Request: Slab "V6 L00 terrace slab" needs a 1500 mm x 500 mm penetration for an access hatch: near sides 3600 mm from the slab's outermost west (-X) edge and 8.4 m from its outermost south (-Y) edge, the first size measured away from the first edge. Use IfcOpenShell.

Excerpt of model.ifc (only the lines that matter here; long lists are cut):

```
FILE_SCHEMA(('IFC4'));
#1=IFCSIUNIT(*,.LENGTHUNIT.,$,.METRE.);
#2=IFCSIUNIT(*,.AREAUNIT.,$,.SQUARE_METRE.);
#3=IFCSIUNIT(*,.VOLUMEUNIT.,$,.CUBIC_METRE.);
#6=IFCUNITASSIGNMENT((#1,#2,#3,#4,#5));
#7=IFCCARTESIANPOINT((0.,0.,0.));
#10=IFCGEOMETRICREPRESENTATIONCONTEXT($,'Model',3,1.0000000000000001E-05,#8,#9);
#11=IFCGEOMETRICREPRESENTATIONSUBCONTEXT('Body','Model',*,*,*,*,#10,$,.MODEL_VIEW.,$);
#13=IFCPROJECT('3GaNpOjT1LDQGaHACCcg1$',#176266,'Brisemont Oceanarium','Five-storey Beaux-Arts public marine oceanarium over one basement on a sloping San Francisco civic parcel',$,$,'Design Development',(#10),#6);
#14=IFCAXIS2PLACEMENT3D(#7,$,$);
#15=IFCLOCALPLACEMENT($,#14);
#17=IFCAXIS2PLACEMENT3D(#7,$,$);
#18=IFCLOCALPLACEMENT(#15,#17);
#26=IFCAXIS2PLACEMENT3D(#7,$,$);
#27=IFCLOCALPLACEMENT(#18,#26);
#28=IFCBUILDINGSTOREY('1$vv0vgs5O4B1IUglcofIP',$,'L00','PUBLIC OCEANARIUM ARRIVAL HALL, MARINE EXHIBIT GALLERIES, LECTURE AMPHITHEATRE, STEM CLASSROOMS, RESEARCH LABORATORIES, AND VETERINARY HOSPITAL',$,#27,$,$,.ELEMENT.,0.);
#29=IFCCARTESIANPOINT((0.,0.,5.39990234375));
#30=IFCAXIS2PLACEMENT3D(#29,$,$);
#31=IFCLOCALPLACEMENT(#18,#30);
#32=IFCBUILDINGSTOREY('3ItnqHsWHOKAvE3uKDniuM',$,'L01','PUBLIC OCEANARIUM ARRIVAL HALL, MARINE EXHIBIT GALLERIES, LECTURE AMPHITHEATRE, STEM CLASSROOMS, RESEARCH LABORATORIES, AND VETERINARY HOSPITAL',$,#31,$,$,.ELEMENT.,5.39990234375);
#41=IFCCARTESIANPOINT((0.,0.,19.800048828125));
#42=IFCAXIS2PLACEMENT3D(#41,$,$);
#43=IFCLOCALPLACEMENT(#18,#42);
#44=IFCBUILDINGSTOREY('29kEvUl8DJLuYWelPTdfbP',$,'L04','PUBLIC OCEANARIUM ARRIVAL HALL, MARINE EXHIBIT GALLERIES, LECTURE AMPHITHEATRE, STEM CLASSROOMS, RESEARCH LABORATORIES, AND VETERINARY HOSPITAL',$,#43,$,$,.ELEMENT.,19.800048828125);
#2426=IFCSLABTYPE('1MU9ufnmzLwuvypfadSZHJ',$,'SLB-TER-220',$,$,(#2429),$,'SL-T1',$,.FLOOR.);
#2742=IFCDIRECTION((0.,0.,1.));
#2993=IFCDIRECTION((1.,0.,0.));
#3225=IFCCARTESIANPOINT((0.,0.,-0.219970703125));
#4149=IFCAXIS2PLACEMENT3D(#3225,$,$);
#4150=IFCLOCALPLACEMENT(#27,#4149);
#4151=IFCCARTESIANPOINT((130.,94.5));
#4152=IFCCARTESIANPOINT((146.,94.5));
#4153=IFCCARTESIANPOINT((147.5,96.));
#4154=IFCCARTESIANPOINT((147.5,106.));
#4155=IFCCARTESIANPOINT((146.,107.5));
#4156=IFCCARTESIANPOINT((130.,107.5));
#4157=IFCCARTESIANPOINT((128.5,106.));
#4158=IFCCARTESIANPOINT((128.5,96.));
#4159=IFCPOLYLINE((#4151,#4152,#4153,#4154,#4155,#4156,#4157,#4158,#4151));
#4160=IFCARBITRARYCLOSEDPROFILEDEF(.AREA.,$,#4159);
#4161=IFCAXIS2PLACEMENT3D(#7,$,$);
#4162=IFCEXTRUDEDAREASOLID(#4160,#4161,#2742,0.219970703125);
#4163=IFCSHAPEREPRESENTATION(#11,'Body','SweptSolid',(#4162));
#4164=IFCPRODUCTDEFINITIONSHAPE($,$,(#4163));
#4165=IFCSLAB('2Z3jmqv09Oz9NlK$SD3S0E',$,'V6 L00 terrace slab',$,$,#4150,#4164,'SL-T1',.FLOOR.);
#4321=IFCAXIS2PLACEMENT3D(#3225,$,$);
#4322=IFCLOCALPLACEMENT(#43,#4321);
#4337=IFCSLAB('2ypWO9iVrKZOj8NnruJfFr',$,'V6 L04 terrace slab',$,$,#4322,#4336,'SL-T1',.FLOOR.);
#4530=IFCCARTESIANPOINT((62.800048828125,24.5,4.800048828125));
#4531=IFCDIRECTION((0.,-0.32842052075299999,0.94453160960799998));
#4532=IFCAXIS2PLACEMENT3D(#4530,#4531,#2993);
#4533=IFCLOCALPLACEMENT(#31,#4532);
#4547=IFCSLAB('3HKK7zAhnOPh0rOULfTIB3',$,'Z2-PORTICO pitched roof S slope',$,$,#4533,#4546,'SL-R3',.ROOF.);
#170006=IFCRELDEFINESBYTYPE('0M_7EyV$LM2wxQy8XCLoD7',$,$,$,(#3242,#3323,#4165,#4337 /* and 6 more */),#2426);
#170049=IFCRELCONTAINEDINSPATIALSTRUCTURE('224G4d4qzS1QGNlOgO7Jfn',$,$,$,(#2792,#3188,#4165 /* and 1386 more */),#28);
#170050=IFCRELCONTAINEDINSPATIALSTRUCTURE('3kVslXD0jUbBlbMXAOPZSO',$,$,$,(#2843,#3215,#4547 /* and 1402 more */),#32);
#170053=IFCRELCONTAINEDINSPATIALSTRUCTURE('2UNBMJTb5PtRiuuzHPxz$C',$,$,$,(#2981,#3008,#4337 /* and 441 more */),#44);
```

```python
import numpy as np
import ifcopenshell
import ifcopenshell.api.feature
import ifcopenshell.api.geometry
import ifcopenshell.api.root
import ifcopenshell.geom
import ifcopenshell.util.placement
import ifcopenshell.util.representation
import ifcopenshell.util.shape
import ifcopenshell.util.unit

model = ifcopenshell.open("model.ifc")
unit_scale = ifcopenshell.util.unit.calculate_unit_scale(model)
settings = ifcopenshell.geom.settings()


def volume(element):
    """Net volume in cubic metres, openings subtracted."""
    shape = ifcopenshell.geom.create_shape(settings, element)
    return ifcopenshell.util.shape.get_volume(shape.geometry)


slab = model.by_guid("2Z3jmqv09Oz9NlK$SD3S0E")
before = volume(slab)

# Extent in the slab's own axes, in metres. The edges named are its -X and -Y sides.
slab_shape = ifcopenshell.geom.create_shape(settings, slab)
vertices = ifcopenshell.util.shape.get_vertices(slab_shape.geometry)
x_min, y_min, bottom = vertices.min(axis=0)
top = vertices[:, 2].max()

opening = ifcopenshell.api.root.create_entity(model, ifc_class="IfcOpeningElement", name="Access hatch opening", predefined_type="OPENING")
context = ifcopenshell.util.representation.get_context(model, "Model", "Body", "MODEL_VIEW")
width, depth = 1.5, 0.5
outline = [(0.0, 0.0), (width, 0.0), (width, depth), (0.0, depth), (0.0, 0.0)]
# Overshoot both faces by 50 mm so the cut is clean.
shape = ifcopenshell.api.geometry.add_slab_representation(
    model, context=context, depth=top - bottom + 0.1, polyline=outline
)
ifcopenshell.api.geometry.assign_representation(model, product=opening, representation=shape)

matrix = ifcopenshell.util.placement.get_local_placement(slab.ObjectPlacement)
matrix[:, 3] = matrix @ np.append(np.array([x_min + 3.6, y_min + 8.4, bottom - 0.05]) / unit_scale, 1.0)
ifcopenshell.api.geometry.edit_object_placement(model, product=opening, matrix=matrix, is_si=False)
ifcopenshell.api.feature.add_feature(model, feature=opening, element=slab)

after = volume(slab)

print(f"slab volume {before:.3f} -> {after:.3f} m3")

model.write("model_edited.ifc")
```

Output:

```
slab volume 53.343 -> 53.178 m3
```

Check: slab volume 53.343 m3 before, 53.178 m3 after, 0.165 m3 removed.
